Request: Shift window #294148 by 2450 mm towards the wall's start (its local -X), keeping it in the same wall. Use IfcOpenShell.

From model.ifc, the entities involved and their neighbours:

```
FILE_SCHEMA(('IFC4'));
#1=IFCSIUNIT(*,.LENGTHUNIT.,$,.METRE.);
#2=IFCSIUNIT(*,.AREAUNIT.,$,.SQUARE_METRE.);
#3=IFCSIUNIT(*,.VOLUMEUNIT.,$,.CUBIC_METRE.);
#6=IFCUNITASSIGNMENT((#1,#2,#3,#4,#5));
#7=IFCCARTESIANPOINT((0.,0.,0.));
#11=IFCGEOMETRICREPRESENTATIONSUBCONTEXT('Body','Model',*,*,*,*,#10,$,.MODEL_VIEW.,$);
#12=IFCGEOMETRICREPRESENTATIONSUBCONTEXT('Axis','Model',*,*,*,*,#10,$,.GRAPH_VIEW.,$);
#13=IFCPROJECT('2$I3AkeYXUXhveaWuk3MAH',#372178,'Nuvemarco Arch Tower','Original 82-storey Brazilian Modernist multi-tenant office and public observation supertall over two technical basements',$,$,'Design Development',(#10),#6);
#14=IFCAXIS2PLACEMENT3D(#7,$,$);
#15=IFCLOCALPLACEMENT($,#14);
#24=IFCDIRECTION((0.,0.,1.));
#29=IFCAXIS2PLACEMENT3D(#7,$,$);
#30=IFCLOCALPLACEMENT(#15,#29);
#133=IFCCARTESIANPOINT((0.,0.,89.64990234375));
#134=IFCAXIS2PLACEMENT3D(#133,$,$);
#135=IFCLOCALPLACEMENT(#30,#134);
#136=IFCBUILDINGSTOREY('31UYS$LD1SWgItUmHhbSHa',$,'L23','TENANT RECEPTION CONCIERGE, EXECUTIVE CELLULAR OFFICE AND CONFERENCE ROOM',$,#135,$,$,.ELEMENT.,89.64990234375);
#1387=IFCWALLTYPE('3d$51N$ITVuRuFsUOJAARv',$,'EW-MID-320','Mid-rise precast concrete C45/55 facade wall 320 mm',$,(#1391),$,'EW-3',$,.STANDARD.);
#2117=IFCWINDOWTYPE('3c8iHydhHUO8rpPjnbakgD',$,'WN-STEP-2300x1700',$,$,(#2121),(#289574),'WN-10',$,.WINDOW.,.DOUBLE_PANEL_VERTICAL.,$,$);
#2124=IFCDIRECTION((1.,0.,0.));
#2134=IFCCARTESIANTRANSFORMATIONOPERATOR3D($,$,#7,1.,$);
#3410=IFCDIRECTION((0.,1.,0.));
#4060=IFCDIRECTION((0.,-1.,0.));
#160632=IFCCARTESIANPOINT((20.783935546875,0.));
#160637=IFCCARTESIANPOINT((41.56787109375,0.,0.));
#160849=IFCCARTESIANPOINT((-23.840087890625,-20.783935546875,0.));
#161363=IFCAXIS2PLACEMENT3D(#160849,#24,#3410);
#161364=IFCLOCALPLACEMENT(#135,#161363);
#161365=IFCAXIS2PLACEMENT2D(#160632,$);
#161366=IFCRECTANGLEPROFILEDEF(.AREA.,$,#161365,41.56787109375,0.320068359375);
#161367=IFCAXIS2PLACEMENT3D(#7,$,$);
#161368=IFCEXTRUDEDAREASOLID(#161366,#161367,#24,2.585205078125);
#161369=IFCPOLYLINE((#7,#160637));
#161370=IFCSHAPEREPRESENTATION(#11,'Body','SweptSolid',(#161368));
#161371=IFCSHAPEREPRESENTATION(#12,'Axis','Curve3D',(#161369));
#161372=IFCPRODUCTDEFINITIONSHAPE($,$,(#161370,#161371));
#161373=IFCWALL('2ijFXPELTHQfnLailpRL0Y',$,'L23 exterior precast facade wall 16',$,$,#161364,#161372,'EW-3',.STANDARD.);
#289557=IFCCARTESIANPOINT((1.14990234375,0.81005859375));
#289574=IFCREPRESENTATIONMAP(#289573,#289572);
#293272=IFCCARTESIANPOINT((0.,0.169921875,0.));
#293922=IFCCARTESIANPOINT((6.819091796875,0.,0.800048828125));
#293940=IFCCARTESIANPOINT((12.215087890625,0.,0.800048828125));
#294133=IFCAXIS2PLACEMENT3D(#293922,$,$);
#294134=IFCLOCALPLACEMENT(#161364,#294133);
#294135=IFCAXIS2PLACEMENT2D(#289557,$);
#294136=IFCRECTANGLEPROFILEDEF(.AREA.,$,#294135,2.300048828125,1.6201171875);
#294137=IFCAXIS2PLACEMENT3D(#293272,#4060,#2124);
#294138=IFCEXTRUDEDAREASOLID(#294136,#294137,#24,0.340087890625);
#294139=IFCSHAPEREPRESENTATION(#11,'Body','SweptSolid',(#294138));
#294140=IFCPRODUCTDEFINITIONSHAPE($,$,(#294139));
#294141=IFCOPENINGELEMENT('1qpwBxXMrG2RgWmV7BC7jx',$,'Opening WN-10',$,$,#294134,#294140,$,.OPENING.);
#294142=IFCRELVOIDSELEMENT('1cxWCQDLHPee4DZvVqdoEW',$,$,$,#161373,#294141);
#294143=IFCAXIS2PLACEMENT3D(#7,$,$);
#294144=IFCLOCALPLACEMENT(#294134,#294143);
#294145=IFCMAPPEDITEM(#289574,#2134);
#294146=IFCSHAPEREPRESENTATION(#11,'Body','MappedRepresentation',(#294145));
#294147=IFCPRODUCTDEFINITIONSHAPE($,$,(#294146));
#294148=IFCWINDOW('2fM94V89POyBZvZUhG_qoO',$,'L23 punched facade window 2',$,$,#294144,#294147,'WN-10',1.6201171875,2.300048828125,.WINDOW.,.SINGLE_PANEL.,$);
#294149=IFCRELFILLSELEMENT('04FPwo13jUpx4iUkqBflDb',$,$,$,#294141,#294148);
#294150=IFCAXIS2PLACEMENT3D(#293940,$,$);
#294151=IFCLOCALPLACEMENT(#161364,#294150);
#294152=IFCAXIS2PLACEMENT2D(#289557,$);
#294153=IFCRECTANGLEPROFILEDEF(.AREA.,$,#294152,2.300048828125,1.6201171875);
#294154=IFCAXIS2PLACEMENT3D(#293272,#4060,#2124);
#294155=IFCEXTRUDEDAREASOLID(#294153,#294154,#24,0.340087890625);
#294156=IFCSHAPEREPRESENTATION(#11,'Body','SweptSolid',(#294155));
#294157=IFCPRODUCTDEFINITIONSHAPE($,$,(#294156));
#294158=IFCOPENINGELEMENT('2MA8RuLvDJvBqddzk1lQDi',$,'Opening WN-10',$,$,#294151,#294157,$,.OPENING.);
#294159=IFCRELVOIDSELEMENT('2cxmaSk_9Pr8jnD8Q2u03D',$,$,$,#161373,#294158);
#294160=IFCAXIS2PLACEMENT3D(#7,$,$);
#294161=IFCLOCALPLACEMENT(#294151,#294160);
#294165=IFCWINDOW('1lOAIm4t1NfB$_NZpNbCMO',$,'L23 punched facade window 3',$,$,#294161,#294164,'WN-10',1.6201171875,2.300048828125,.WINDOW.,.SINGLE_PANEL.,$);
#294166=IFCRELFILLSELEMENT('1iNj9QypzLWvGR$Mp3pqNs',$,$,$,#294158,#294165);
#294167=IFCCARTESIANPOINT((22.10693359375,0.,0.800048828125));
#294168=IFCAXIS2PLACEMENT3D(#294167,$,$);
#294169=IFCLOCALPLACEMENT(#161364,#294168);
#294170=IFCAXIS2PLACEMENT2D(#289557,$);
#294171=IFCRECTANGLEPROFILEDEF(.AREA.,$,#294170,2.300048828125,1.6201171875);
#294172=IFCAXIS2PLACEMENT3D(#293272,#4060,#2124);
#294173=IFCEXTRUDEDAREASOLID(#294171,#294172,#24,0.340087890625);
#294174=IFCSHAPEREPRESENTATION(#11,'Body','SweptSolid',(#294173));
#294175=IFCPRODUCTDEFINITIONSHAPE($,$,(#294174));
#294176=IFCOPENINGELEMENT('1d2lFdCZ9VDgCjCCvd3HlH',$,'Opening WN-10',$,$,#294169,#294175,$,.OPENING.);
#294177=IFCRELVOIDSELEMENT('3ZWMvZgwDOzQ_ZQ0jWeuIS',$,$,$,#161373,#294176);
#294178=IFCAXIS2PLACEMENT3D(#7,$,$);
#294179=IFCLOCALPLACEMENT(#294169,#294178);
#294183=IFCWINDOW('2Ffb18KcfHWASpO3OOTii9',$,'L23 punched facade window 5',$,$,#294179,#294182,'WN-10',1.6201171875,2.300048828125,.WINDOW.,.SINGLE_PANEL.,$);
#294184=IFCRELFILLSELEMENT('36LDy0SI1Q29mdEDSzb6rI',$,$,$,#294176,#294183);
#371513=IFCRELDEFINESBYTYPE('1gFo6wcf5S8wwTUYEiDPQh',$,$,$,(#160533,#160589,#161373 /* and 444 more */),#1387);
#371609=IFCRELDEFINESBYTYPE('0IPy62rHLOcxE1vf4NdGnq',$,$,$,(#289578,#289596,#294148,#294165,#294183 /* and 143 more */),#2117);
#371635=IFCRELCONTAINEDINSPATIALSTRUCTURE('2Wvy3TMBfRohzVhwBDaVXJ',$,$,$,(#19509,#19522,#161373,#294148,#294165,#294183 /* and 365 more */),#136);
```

```python
import ifcopenshell
import ifcopenshell.api.geometry
import ifcopenshell.util.placement

model = ifcopenshell.open("model.ifc")

window = model.by_guid("2fM94V89POyBZvZUhG_qoO")
opening = window.FillsVoids[0].RelatingOpeningElement
wall = opening.VoidsElements[0].RelatingBuildingElement

wall_matrix = ifcopenshell.util.placement.get_local_placement(wall.ObjectPlacement)
shift = wall_matrix[:3, 0] * -2.45
before = ifcopenshell.util.placement.get_local_placement(window.ObjectPlacement)[:3, 3].copy()

# The window is placed relative to its opening, so it follows when the opening moves.
matrix = ifcopenshell.util.placement.get_local_placement(opening.ObjectPlacement)
matrix[:3, 3] += shift
ifcopenshell.api.geometry.edit_object_placement(
    model, product=opening, matrix=matrix, is_si=False, should_transform_children=True
)

after = ifcopenshell.util.placement.get_local_placement(window.ObjectPlacement)[:3, 3]
print("window moved by", (after - before).round(3) + 0.0)

model.write("model_v2.ifc")
```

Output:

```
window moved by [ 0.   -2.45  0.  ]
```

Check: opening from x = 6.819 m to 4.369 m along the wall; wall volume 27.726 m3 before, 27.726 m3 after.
